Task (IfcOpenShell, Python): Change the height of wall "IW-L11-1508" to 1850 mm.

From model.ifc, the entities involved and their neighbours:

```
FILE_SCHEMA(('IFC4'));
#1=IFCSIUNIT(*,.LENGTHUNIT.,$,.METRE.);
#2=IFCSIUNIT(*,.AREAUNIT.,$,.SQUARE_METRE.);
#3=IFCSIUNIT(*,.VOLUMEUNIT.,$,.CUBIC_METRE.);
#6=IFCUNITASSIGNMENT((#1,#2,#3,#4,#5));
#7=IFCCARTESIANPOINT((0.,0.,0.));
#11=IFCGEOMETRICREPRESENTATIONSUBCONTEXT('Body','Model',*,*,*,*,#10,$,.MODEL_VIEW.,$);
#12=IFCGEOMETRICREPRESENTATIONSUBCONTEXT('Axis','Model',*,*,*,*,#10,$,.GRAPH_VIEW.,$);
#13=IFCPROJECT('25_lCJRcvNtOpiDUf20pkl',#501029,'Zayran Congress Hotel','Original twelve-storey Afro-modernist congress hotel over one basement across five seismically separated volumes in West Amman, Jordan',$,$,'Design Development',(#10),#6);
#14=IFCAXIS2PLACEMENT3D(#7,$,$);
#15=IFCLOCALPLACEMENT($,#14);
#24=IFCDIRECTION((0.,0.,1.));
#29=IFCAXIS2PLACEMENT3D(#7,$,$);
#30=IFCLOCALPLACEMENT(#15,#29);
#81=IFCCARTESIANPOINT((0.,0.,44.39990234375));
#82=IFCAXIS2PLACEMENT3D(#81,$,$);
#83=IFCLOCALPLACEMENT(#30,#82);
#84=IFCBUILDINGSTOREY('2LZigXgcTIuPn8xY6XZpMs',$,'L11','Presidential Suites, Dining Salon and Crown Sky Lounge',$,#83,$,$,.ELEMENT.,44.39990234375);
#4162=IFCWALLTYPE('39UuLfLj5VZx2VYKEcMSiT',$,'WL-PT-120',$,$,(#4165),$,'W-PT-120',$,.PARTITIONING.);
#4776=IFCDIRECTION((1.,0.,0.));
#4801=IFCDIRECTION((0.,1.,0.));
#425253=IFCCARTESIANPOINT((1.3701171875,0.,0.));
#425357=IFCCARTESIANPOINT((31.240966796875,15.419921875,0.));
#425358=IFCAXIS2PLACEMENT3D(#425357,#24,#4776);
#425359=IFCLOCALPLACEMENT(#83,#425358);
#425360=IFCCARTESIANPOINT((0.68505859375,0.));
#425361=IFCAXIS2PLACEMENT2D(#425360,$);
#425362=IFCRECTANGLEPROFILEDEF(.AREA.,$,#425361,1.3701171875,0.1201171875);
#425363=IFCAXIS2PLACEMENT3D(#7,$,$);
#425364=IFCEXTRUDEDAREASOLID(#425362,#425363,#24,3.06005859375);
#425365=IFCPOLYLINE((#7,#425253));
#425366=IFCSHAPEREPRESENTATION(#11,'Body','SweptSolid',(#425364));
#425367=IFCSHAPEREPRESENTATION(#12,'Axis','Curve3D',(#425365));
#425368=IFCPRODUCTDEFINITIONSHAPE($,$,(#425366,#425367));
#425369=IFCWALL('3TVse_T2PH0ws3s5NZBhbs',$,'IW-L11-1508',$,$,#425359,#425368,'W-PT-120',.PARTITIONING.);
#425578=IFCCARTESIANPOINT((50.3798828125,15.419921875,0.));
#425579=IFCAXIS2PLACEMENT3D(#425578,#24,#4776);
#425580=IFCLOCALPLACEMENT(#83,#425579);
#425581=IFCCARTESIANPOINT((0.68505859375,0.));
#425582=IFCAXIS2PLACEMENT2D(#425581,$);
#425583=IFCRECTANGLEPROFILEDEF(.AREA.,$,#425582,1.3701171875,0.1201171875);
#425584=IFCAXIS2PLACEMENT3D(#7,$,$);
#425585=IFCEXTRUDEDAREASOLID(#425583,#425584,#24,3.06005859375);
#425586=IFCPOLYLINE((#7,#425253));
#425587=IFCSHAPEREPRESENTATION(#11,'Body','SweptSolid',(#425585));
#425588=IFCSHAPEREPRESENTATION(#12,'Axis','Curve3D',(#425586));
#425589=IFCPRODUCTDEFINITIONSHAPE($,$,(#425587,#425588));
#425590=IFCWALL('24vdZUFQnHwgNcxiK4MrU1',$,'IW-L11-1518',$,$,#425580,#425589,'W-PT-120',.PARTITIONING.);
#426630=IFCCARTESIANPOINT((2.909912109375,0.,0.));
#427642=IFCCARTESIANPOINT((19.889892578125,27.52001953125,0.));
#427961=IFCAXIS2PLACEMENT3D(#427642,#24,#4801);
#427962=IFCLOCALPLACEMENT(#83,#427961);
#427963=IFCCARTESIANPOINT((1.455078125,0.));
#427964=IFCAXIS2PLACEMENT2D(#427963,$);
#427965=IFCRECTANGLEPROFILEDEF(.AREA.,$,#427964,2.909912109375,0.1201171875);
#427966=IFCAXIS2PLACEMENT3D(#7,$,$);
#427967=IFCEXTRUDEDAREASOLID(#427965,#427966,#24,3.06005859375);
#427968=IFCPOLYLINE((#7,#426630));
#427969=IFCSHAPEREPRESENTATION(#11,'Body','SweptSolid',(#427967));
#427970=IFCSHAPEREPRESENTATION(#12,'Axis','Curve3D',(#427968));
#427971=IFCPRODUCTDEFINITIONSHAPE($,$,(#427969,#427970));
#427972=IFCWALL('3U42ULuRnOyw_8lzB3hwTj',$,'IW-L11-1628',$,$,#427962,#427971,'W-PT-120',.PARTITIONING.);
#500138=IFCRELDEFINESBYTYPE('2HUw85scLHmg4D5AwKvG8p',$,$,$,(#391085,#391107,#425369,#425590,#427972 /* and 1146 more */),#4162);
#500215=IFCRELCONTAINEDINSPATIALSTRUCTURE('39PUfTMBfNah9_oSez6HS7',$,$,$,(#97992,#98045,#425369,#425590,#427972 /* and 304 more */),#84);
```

```python
import ifcopenshell
import ifcopenshell.geom
import ifcopenshell.util.representation
import ifcopenshell.util.shape
import ifcopenshell.util.unit

model = ifcopenshell.open("model.ifc")
unit_scale = ifcopenshell.util.unit.calculate_unit_scale(model)
settings = ifcopenshell.geom.settings()


def volume(element):
    """Net volume in cubic metres, openings subtracted."""
    shape = ifcopenshell.geom.create_shape(settings, element)
    return ifcopenshell.util.shape.get_volume(shape.geometry)


wall = model.by_guid("3TVse_T2PH0ws3s5NZBhbs")
before = volume(wall)

body = ifcopenshell.util.representation.get_representation(wall, "Model", "Body")
solid = body.Items[0]
old_height = solid.Depth
solid.Depth = 1.85 / unit_scale
after = volume(wall)

print(f"height {old_height:g} -> {solid.Depth:g}, volume {before:.3f} -> {after:.3f} m3")

model.write("model_updated.ifc")
```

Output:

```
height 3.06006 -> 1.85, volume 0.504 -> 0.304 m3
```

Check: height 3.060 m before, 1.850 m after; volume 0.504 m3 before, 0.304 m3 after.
